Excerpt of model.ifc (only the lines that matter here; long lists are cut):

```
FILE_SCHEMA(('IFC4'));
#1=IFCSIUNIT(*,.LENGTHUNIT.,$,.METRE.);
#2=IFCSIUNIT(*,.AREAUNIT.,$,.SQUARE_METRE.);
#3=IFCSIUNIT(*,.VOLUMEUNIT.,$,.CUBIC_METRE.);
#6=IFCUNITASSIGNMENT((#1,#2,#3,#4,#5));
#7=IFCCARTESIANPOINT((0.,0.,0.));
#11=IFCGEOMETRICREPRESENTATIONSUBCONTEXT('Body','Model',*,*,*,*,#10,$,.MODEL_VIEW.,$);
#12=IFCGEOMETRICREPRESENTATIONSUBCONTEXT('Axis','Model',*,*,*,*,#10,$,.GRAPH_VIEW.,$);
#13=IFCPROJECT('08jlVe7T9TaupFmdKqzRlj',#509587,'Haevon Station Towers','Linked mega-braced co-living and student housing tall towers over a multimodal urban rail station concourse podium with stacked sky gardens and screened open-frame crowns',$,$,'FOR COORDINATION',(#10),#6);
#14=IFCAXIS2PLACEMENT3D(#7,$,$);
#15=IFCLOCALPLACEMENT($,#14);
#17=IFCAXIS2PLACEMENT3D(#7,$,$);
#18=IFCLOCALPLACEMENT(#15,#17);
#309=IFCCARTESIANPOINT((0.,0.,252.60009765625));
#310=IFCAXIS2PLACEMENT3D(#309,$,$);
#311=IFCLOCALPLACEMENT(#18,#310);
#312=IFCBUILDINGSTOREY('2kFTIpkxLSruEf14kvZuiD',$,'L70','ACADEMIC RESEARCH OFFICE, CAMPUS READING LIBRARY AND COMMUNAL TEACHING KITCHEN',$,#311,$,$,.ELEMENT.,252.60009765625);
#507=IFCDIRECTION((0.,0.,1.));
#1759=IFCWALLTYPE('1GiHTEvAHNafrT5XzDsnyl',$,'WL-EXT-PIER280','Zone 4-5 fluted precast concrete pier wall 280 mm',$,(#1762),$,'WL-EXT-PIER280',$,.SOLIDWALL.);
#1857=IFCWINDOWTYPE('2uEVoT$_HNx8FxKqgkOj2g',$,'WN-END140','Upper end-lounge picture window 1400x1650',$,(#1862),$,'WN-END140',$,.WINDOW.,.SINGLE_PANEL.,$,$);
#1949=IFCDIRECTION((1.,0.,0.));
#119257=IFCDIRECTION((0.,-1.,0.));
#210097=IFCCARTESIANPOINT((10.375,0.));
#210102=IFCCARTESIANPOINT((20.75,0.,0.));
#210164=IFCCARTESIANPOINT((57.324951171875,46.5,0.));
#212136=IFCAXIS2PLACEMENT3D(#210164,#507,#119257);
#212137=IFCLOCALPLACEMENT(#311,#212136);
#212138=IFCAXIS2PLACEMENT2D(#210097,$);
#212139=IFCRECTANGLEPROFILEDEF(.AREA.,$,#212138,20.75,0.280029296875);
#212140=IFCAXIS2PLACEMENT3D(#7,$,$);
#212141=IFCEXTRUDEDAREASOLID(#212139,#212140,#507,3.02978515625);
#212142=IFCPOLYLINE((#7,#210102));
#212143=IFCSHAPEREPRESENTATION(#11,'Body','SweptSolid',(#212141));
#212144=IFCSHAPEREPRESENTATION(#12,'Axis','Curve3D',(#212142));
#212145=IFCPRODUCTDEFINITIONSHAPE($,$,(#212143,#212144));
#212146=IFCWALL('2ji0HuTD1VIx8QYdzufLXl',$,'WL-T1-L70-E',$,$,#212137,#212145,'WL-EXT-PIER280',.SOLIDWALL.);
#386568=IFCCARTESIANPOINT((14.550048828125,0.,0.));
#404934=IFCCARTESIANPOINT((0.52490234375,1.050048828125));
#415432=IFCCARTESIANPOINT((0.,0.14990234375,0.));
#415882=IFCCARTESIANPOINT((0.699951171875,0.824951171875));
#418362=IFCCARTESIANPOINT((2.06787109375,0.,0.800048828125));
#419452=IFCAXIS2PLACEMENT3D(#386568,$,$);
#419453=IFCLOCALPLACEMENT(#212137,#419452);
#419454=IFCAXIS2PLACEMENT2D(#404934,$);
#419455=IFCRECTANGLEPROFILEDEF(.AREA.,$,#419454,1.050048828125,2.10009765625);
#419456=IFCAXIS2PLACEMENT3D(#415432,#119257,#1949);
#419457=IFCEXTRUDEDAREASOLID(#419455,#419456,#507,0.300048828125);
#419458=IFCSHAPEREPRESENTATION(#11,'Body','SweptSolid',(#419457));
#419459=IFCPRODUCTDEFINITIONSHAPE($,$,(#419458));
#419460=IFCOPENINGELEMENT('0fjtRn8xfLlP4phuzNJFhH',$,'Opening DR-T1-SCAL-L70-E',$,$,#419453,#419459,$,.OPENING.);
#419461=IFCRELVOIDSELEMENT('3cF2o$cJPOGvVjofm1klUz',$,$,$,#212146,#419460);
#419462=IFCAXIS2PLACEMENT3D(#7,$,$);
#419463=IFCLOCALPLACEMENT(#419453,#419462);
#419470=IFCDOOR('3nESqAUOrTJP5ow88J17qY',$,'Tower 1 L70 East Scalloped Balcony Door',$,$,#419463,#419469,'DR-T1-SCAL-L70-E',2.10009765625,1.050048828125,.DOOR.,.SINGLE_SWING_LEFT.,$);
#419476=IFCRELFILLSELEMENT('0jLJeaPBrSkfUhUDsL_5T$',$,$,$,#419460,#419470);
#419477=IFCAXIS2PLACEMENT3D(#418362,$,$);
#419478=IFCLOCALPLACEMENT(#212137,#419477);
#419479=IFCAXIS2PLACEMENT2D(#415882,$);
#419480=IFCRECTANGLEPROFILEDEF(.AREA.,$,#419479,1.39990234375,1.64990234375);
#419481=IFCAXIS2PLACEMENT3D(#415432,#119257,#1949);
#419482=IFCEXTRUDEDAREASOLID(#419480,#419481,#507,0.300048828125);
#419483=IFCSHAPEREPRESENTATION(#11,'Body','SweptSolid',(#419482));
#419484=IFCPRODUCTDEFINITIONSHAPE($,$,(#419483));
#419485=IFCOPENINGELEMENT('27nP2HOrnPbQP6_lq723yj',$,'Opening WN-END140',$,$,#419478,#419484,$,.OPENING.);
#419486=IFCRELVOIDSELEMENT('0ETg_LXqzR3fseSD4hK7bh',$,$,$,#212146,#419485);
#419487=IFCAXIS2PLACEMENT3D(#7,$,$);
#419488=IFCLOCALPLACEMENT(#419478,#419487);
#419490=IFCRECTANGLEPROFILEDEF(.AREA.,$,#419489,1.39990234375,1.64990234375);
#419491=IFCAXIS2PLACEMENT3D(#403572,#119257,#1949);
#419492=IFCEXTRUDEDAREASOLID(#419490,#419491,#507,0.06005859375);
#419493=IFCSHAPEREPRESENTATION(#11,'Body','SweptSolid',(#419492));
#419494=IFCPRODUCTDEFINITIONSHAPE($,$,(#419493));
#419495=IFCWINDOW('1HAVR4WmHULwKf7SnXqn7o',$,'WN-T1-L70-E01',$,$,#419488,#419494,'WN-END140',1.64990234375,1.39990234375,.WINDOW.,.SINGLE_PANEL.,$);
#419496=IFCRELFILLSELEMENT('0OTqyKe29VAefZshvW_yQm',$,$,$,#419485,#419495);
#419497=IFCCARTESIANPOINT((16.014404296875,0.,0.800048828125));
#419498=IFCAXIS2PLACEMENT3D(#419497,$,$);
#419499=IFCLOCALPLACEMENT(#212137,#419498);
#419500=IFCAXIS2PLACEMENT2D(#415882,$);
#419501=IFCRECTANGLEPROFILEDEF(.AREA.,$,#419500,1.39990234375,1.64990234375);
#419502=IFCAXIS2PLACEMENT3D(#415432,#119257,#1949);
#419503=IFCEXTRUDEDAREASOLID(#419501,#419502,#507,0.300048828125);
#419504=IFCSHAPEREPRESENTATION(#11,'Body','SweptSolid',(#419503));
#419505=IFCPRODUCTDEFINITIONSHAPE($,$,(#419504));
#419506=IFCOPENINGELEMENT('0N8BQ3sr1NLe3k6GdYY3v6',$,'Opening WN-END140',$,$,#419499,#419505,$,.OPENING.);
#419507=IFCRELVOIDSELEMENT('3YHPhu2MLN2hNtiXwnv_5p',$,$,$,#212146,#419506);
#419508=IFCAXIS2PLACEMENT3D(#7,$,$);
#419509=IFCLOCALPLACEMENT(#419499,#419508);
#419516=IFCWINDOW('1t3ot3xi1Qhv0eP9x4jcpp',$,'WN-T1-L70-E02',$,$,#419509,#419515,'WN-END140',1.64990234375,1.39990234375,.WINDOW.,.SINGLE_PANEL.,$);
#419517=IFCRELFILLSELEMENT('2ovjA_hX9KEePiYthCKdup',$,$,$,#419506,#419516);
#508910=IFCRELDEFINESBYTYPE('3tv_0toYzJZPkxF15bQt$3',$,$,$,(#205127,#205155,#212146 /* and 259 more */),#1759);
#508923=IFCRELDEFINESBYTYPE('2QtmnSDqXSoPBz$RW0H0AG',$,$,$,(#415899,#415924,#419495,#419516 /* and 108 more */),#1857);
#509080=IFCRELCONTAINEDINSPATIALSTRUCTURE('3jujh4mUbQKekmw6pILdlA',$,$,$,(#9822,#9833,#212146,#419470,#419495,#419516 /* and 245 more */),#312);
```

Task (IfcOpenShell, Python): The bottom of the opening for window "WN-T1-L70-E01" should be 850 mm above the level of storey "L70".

```python
import numpy as np
import ifcopenshell
import ifcopenshell.api.geometry
import ifcopenshell.geom
import ifcopenshell.util.element
import ifcopenshell.util.placement
import ifcopenshell.util.shape
import ifcopenshell.util.unit

model = ifcopenshell.open("model.ifc")
unit_scale = ifcopenshell.util.unit.calculate_unit_scale(model)

window = model.by_id(419495)
opening = window.FillsVoids[0].RelatingOpeningElement
storey = ifcopenshell.util.element.get_container(window, ifc_class="IfcBuildingStorey")
level = ifcopenshell.util.placement.get_local_placement(storey.ObjectPlacement)[2, 3]

# The opening's origin need not be at the sill, so measure its lowest point.
shape = ifcopenshell.geom.create_shape(ifcopenshell.geom.settings(), opening)
bottom = ifcopenshell.util.shape.get_shape_bottom_elevation(shape, shape.geometry) / unit_scale
dz = level + 0.85 - bottom

shift = np.array([0.0, 0.0, dz])
# The window is placed relative to its opening, so it follows when the opening moves.
matrix = ifcopenshell.util.placement.get_local_placement(opening.ObjectPlacement)
matrix[:3, 3] += shift
ifcopenshell.api.geometry.edit_object_placement(
    model, product=opening, matrix=matrix, is_si=False, should_transform_children=True
)

print(f"moved by {dz * unit_scale:+.3f} m")

model.write("model_rev.ifc")
```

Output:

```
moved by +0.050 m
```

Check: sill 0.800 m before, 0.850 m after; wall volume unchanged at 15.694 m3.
